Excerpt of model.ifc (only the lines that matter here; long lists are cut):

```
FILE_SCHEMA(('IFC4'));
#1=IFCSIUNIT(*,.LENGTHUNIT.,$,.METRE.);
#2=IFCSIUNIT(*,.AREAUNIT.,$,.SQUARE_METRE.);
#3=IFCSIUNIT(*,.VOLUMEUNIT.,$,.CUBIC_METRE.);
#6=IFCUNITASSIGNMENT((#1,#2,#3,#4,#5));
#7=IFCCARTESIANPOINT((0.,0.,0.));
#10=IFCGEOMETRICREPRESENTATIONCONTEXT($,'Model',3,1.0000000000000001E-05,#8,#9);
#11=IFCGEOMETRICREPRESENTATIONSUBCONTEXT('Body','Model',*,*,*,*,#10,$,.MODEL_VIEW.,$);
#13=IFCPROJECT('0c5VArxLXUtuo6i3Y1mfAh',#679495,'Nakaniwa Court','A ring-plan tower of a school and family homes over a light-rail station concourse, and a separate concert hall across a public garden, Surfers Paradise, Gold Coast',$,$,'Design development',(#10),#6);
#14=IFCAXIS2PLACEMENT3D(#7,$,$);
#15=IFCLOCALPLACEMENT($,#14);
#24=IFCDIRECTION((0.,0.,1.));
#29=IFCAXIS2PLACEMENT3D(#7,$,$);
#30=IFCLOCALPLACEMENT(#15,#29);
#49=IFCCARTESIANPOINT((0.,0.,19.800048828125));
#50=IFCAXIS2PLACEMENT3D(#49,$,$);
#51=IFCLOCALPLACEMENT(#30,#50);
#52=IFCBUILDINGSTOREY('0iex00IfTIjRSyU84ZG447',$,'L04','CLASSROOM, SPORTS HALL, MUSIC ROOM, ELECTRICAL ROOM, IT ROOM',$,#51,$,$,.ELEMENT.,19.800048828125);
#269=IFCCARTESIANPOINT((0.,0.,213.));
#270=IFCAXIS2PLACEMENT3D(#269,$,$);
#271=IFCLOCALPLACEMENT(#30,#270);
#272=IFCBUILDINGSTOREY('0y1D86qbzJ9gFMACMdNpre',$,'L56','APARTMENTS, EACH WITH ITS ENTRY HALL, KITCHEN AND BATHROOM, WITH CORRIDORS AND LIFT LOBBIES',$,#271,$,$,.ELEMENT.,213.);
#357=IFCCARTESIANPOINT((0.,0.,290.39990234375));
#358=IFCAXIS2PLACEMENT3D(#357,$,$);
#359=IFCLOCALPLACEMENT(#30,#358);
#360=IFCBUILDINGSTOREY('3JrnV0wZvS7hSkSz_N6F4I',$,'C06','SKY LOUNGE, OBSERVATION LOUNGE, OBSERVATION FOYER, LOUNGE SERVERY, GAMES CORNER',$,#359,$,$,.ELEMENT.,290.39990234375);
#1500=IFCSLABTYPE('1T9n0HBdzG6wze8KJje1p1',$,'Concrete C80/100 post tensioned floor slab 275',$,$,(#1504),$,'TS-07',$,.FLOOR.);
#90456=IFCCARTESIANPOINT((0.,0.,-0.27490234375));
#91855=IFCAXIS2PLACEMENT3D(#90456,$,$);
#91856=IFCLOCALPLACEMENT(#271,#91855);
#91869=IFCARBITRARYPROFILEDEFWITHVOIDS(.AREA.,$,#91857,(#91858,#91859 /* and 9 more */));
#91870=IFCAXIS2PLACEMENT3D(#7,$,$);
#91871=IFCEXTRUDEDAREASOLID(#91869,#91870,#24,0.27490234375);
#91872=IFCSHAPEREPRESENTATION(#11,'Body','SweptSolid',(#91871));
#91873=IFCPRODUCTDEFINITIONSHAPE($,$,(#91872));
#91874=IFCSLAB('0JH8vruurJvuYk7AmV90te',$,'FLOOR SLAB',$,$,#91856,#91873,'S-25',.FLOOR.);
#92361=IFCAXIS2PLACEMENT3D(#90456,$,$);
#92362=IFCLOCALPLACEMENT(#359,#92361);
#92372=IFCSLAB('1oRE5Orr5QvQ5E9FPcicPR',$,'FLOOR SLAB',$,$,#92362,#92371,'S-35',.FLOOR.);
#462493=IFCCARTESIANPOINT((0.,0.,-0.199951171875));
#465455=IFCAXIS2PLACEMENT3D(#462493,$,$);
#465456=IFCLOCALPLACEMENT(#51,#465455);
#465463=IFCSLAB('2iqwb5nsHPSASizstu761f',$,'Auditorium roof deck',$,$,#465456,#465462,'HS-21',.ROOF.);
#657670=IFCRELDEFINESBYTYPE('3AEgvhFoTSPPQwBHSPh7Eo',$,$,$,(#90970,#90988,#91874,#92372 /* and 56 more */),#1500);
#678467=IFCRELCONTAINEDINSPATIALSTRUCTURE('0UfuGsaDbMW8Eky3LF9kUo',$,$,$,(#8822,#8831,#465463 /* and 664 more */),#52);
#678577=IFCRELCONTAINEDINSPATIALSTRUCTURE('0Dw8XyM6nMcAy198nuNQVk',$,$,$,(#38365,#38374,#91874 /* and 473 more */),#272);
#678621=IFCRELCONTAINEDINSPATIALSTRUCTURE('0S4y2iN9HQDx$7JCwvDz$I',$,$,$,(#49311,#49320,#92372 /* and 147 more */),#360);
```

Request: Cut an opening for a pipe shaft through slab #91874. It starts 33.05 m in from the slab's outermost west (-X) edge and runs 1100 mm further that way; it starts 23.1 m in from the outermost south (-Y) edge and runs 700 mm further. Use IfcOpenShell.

```python
import numpy as np
import ifcopenshell
import ifcopenshell.api.feature
import ifcopenshell.api.geometry
import ifcopenshell.api.root
import ifcopenshell.geom
import ifcopenshell.util.placement
import ifcopenshell.util.representation
import ifcopenshell.util.shape
import ifcopenshell.util.unit

model = ifcopenshell.open("model.ifc")
unit_scale = ifcopenshell.util.unit.calculate_unit_scale(model)
settings = ifcopenshell.geom.settings()


def volume(element):
    """Net volume in cubic metres, openings subtracted."""
    shape = ifcopenshell.geom.create_shape(settings, element)
    return ifcopenshell.util.shape.get_volume(shape.geometry)


slab = model.by_guid("0JH8vruurJvuYk7AmV90te")
before = volume(slab)

# Extent in the slab's own axes, in metres. The edges named are its -X and -Y sides.
slab_shape = ifcopenshell.geom.create_shape(settings, slab)
vertices = ifcopenshell.util.shape.get_vertices(slab_shape.geometry)
x_min, y_min, bottom = vertices.min(axis=0)
top = vertices[:, 2].max()

opening = ifcopenshell.api.root.create_entity(model, ifc_class="IfcOpeningElement", name="Pipe shaft opening", predefined_type="OPENING")
context = ifcopenshell.util.representation.get_context(model, "Model", "Body", "MODEL_VIEW")
width, depth = 1.1, 0.7
outline = [(0.0, 0.0), (width, 0.0), (width, depth), (0.0, depth), (0.0, 0.0)]
# Overshoot both faces by 50 mm so the cut is clean.
shape = ifcopenshell.api.geometry.add_slab_representation(
    model, context=context, depth=top - bottom + 0.1, polyline=outline
)
ifcopenshell.api.geometry.assign_representation(model, product=opening, representation=shape)

matrix = ifcopenshell.util.placement.get_local_placement(slab.ObjectPlacement)
matrix[:, 3] = matrix @ np.append(np.array([x_min + 33.05, y_min + 23.1, bottom - 0.05]) / unit_scale, 1.0)
ifcopenshell.api.geometry.edit_object_placement(model, product=opening, matrix=matrix, is_si=False)
ifcopenshell.api.feature.add_feature(model, feature=opening, element=slab)

after = volume(slab)

print(f"slab volume {before:.3f} -> {after:.3f} m3")

model.write("model-out.ifc")
```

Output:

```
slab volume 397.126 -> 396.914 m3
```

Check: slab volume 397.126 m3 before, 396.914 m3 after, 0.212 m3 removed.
